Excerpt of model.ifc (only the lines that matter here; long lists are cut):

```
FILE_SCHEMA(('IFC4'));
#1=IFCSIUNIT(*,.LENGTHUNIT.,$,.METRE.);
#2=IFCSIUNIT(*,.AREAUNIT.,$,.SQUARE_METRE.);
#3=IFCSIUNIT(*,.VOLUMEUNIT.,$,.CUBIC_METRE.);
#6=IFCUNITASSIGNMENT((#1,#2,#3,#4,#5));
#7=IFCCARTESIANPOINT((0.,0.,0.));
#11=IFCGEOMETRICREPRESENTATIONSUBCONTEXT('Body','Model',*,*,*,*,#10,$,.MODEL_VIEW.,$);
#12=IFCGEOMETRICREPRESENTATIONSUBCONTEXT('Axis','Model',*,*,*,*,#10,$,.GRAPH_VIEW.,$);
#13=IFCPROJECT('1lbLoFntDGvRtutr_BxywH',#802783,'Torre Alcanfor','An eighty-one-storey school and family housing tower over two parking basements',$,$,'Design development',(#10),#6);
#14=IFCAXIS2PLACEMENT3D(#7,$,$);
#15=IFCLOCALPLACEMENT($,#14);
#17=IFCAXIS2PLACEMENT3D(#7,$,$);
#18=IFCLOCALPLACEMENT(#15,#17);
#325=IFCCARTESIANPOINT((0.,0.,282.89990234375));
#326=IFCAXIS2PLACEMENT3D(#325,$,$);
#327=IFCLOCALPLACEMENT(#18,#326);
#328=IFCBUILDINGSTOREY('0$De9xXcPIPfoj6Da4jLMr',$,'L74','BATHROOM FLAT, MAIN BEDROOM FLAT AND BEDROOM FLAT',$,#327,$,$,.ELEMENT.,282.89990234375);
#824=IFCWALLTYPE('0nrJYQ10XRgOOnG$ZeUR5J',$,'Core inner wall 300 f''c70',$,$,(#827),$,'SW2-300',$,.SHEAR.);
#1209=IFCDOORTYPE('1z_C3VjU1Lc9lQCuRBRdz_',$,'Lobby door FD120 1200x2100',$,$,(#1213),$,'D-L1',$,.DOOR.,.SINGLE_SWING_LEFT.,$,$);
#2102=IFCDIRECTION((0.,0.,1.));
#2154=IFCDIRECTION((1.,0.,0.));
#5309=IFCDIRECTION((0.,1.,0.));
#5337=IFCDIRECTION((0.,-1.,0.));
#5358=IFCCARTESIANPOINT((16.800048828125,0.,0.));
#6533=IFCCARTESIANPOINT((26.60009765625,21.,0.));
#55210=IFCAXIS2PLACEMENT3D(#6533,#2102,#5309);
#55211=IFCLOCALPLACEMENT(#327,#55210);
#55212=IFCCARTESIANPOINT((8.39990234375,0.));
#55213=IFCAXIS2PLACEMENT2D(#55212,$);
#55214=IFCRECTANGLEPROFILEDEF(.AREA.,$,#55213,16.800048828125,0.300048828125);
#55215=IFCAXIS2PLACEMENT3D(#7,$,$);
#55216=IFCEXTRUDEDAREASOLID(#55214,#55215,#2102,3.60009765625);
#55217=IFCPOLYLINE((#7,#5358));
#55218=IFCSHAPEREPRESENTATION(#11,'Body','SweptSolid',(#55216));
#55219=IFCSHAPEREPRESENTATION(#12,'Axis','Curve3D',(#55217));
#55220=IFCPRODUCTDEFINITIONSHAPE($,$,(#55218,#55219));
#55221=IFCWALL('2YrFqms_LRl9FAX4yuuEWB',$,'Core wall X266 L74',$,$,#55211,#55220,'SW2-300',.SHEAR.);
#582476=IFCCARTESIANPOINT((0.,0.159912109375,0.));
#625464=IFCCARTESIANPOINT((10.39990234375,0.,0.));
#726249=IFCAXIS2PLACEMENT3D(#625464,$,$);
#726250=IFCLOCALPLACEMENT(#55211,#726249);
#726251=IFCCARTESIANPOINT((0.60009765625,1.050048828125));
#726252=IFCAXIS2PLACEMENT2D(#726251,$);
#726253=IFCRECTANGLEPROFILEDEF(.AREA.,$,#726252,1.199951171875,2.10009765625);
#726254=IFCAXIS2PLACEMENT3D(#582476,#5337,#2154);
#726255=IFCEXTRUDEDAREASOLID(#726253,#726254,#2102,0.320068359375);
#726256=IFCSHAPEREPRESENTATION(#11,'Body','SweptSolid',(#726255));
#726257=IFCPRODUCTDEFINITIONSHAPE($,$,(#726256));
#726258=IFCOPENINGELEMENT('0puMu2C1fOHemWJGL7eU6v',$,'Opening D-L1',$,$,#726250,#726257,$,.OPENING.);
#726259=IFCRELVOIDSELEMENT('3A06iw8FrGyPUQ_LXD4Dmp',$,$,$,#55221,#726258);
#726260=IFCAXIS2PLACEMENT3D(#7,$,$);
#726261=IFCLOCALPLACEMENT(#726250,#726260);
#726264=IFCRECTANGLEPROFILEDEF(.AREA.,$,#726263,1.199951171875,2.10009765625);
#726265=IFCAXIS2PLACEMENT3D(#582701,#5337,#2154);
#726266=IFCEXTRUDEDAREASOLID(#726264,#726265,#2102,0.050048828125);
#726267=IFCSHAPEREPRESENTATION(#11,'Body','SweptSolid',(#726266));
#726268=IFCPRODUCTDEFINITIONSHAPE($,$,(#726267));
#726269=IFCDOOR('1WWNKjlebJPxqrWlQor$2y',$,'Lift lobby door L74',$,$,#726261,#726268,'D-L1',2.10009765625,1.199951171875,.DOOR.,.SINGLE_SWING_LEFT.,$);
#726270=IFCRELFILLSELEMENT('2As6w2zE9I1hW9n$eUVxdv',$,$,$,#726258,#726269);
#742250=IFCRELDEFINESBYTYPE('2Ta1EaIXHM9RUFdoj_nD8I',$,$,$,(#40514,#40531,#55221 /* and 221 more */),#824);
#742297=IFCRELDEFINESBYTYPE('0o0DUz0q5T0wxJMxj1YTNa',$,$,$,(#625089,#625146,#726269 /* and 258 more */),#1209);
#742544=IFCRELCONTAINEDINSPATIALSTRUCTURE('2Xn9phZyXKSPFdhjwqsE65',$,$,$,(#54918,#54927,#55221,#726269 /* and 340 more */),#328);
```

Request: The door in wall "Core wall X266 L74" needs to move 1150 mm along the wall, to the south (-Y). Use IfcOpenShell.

```python
import ifcopenshell
import ifcopenshell.api.geometry
import ifcopenshell.util.placement
import ifcopenshell.util.unit

model = ifcopenshell.open("model.ifc")
unit_scale = ifcopenshell.util.unit.calculate_unit_scale(model)

door = model.by_guid("1WWNKjlebJPxqrWlQor$2y")
opening = door.FillsVoids[0].RelatingOpeningElement
wall = opening.VoidsElements[0].RelatingBuildingElement

wall_matrix = ifcopenshell.util.placement.get_local_placement(wall.ObjectPlacement)
shift = wall_matrix[:3, 0] * -1.15 / unit_scale
before = ifcopenshell.util.placement.get_local_placement(door.ObjectPlacement)[:3, 3].copy()

# The door is placed relative to its opening, so it follows when the opening moves.
matrix = ifcopenshell.util.placement.get_local_placement(opening.ObjectPlacement)
matrix[:3, 3] += shift
ifcopenshell.api.geometry.edit_object_placement(
    model, product=opening, matrix=matrix, is_si=False, should_transform_children=True
)

after = ifcopenshell.util.placement.get_local_placement(door.ObjectPlacement)[:3, 3]
print("door moved by", (after - before).round(3) + 0.0)

model.write("model_v2.ifc")
```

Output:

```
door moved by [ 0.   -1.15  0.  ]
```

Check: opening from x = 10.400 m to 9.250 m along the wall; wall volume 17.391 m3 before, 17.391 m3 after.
